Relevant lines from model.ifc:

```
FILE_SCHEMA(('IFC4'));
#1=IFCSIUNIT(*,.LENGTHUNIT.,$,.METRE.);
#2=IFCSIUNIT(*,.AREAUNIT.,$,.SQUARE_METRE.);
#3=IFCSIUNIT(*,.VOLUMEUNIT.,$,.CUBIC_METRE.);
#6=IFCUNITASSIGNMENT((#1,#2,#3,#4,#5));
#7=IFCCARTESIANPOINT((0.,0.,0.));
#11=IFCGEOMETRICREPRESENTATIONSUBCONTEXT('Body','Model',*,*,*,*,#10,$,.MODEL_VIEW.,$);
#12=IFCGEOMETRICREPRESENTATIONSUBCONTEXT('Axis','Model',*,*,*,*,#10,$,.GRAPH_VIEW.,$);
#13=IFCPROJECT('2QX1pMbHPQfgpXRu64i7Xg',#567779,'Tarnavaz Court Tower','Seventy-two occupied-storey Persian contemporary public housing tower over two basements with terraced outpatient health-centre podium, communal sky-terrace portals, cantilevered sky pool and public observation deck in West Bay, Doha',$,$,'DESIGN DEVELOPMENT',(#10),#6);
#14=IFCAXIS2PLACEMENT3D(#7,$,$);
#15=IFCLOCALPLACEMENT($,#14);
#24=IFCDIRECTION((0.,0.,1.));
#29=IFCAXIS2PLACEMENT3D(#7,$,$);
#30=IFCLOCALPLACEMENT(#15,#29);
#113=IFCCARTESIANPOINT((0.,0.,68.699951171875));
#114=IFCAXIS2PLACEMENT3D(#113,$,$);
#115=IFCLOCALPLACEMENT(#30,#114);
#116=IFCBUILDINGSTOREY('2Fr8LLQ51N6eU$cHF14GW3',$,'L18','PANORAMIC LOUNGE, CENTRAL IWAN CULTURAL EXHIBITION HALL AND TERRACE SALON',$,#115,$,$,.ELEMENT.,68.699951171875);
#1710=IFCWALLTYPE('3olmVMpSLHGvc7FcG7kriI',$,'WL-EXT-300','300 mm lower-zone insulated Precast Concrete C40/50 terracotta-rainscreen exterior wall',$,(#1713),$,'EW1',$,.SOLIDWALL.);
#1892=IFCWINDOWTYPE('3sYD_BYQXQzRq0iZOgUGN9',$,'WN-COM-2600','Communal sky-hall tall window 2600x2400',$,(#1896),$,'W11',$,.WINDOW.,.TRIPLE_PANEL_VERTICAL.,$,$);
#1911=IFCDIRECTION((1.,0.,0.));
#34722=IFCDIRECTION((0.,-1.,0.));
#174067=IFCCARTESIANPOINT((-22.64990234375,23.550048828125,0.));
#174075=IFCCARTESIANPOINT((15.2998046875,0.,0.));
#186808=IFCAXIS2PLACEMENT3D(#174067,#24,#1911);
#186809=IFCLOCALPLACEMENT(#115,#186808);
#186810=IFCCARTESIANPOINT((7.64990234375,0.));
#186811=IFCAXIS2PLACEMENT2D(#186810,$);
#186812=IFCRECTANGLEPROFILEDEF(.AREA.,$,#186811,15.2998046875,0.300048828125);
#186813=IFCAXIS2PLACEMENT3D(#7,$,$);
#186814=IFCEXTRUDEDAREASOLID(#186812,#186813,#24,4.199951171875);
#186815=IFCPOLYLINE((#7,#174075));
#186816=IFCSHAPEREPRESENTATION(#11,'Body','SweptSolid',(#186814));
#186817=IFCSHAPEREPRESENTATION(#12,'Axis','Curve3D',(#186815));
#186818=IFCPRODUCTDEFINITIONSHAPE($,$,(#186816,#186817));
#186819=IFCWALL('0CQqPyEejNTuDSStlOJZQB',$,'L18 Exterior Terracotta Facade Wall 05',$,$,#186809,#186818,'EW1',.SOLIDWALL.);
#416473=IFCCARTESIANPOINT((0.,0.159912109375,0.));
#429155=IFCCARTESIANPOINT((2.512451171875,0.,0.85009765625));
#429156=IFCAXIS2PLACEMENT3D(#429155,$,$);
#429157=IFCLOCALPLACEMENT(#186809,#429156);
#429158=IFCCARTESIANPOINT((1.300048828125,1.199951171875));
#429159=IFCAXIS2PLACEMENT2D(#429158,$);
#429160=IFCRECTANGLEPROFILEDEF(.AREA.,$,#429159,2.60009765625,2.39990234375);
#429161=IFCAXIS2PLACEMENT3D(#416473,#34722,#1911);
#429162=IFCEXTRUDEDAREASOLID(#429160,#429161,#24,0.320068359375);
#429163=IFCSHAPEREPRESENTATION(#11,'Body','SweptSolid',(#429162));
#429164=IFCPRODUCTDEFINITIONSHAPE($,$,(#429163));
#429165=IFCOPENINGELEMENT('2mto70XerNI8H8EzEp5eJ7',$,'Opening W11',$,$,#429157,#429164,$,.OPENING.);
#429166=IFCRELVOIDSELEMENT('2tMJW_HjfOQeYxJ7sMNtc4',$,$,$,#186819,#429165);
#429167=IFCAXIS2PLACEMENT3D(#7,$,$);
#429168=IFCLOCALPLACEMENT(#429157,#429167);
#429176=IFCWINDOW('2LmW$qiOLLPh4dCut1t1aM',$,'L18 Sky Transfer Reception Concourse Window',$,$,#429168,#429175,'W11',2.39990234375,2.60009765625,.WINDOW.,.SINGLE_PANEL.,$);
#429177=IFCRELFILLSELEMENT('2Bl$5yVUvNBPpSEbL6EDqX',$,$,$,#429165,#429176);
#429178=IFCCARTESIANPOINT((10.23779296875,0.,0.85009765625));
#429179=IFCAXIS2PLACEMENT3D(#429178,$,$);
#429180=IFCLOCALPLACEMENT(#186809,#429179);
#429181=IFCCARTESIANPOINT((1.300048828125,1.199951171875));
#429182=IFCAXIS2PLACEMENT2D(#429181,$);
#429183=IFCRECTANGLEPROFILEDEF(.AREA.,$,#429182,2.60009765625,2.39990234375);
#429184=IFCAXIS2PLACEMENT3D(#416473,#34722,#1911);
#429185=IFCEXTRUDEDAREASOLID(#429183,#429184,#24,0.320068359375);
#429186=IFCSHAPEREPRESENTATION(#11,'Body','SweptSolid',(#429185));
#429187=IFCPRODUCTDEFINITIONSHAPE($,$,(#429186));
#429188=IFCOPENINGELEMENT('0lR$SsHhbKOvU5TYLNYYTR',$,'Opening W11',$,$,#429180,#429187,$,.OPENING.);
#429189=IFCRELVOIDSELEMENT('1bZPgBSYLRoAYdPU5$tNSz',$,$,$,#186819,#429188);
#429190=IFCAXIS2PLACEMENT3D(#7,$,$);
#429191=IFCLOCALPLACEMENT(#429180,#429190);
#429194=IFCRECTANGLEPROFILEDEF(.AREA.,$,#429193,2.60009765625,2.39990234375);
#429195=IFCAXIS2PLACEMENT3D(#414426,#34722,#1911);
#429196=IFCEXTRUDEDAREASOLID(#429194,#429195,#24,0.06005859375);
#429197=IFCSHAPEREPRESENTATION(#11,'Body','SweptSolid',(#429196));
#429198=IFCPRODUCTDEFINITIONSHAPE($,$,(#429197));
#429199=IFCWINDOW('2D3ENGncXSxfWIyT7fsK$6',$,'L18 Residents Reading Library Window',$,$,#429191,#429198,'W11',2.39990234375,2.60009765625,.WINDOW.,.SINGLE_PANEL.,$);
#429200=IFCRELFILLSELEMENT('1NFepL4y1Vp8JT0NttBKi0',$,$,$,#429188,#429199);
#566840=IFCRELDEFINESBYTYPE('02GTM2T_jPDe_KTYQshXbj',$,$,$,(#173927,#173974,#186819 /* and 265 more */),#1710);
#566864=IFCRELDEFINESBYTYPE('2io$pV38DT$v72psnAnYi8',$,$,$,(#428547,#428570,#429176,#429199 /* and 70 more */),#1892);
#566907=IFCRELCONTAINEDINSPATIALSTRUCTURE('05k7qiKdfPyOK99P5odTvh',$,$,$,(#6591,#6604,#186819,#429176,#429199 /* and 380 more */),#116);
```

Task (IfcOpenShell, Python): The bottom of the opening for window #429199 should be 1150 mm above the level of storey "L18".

```python
import numpy as np
import ifcopenshell
import ifcopenshell.api.geometry
import ifcopenshell.geom
import ifcopenshell.util.element
import ifcopenshell.util.placement
import ifcopenshell.util.shape
import ifcopenshell.util.unit

model = ifcopenshell.open("model.ifc")
unit_scale = ifcopenshell.util.unit.calculate_unit_scale(model)

window = model.by_id(429199)
opening = window.FillsVoids[0].RelatingOpeningElement
storey = ifcopenshell.util.element.get_container(window, ifc_class="IfcBuildingStorey")
level = ifcopenshell.util.placement.get_local_placement(storey.ObjectPlacement)[2, 3]

# The opening's origin need not be at the sill, so measure its lowest point.
shape = ifcopenshell.geom.create_shape(ifcopenshell.geom.settings(), opening)
bottom = ifcopenshell.util.shape.get_shape_bottom_elevation(shape, shape.geometry) / unit_scale
dz = level + 1.15 / unit_scale - bottom

shift = np.array([0.0, 0.0, dz])
# The window is placed relative to its opening, so it follows when the opening moves.
matrix = ifcopenshell.util.placement.get_local_placement(opening.ObjectPlacement)
matrix[:3, 3] += shift
ifcopenshell.api.geometry.edit_object_placement(
    model, product=opening, matrix=matrix, is_si=False, should_transform_children=True
)

print(f"moved by {dz * unit_scale:+.3f} m")

model.write("model_rev.ifc")
```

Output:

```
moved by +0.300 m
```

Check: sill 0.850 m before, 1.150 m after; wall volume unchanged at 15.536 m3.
